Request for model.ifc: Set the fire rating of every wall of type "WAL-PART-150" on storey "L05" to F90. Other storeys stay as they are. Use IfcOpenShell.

First a look at what the model holds.

```python
import ifcopenshell
import ifcopenshell.util.element

model = ifcopenshell.open("model.ifc")
print(model.schema)
storey = next(s for s in model.by_type("IfcBuildingStorey") if s.Name == "L05")
walls = [e for e in ifcopenshell.util.element.get_decomposition(storey) if e.is_a("IfcWall")]
seen = {}
for e in walls:
    element_type = ifcopenshell.util.element.get_type(e)
    key = (element_type.Name if element_type != e and element_type else None, ifcopenshell.util.element.get_pset(e, "Pset_WallCommon", "FireRating"))
    seen[key] = seen.get(key, 0) + 1
for (name, value), count in sorted(seen.items(), key=str):
    print(count, "x", name, "|", value)
```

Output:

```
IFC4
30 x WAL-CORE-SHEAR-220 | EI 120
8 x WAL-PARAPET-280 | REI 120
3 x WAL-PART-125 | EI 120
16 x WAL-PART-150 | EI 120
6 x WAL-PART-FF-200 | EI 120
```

```python
import ifcopenshell
import ifcopenshell.api.pset
import ifcopenshell.util.element

model = ifcopenshell.open("model.ifc")

storey = next(s for s in model.by_type("IfcBuildingStorey") if s.Name == "L05")
walls = [e for e in ifcopenshell.util.element.get_decomposition(storey) if e.is_a("IfcWall")]

count = 0
for e in walls:
    element_type = ifcopenshell.util.element.get_type(e)
    if element_type in (None, e) or element_type.Name != "WAL-PART-150":
        continue
    # add_pset returns the element's existing set when there is one.
    pset = ifcopenshell.api.pset.add_pset(model, product=e, name="Pset_WallCommon")
    ifcopenshell.api.pset.edit_pset(model, pset=pset, properties={"FireRating": "F90"})
    count += 1

print(count, "walls updated")

model.write("model-out.ifc")
```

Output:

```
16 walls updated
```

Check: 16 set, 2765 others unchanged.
